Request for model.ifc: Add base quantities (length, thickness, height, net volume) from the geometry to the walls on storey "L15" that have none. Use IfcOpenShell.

First a look at what the model holds.

```python
import ifcopenshell
import ifcopenshell.util.element
import ifcopenshell.util.unit

model = ifcopenshell.open("model.ifc")
print(model.schema)
for unit_type in ("LENGTHUNIT", "AREAUNIT", "VOLUMEUNIT"):
    print(unit_type, ifcopenshell.util.unit.calculate_unit_scale(model, unit_type))
storey = next(s for s in model.by_type("IfcBuildingStorey") if s.Name == "L15")
walls = [e for e in ifcopenshell.util.element.get_decomposition(storey) if e.is_a("IfcWall")]
for e in sorted(walls, key=lambda e: e.id()):
    print(e.id(), e.is_a(), e.Name, list(ifcopenshell.util.element.get_psets(e, qtos_only=True)), sep=" | ")
```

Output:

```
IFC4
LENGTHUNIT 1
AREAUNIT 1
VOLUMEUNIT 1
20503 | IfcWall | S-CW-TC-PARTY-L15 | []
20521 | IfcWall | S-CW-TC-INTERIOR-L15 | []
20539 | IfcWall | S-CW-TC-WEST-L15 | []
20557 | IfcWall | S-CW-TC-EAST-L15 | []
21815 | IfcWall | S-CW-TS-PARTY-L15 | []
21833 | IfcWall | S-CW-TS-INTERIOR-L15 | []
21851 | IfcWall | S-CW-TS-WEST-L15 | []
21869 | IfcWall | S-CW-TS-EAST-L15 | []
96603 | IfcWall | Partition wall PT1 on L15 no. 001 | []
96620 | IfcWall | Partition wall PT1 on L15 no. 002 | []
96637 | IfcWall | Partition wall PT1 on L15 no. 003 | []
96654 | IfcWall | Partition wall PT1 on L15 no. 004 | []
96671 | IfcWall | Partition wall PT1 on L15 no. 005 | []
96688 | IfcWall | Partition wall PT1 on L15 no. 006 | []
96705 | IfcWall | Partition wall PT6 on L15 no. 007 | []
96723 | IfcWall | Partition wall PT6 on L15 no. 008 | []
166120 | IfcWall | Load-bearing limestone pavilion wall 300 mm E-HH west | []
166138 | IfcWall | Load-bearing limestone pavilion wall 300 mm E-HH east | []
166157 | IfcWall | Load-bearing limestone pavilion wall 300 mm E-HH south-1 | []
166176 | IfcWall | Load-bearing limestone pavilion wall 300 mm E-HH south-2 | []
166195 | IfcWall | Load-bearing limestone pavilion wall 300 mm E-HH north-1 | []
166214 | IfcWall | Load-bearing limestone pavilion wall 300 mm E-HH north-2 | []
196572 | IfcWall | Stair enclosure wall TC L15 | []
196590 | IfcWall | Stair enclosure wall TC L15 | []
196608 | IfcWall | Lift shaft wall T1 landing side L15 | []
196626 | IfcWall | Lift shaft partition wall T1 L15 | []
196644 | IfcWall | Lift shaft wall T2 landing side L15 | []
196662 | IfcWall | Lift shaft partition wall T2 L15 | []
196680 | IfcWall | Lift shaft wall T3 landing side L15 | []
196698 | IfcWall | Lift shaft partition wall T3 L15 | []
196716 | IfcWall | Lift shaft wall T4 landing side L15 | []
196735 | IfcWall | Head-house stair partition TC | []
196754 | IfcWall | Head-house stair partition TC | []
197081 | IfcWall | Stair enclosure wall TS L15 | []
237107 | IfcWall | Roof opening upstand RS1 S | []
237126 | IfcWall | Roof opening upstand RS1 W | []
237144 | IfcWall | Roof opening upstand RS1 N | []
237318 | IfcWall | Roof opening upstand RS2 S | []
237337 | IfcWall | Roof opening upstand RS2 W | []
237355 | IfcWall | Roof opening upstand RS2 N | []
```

```python
import ifcopenshell
import ifcopenshell.api.pset
import ifcopenshell.geom
import ifcopenshell.util.element
import ifcopenshell.util.shape
import ifcopenshell.util.unit

model = ifcopenshell.open("model.ifc")
unit_scale = ifcopenshell.util.unit.calculate_unit_scale(model)
volume_scale = ifcopenshell.util.unit.calculate_unit_scale(model, "VOLUMEUNIT")
settings = ifcopenshell.geom.settings()

storey = next(s for s in model.by_type("IfcBuildingStorey") if s.Name == "L15")
walls = [e for e in ifcopenshell.util.element.get_decomposition(storey) if e.is_a("IfcWall")]

for e in sorted(walls, key=lambda e: e.id()):
    if ifcopenshell.util.element.get_psets(e, qtos_only=True, should_inherit=False):
        continue
    # Geometry comes back in metres, in the element's own axes.
    shape = ifcopenshell.geom.create_shape(settings, e)
    values = {
        "Length": ifcopenshell.util.shape.get_x(shape.geometry) / unit_scale,
        "Width": ifcopenshell.util.shape.get_y(shape.geometry) / unit_scale,
        "Height": ifcopenshell.util.shape.get_z(shape.geometry) / unit_scale,
        "NetVolume": ifcopenshell.util.shape.get_volume(shape.geometry) / volume_scale,
    }
    qto = ifcopenshell.api.pset.add_qto(model, product=e, name="Qto_WallBaseQuantities")
    ifcopenshell.api.pset.edit_qto(model, qto=qto, properties=values)
    print(e.id(), {k: round(v, 3) for k, v in values.items()})

model.write("model_v2.ifc")
```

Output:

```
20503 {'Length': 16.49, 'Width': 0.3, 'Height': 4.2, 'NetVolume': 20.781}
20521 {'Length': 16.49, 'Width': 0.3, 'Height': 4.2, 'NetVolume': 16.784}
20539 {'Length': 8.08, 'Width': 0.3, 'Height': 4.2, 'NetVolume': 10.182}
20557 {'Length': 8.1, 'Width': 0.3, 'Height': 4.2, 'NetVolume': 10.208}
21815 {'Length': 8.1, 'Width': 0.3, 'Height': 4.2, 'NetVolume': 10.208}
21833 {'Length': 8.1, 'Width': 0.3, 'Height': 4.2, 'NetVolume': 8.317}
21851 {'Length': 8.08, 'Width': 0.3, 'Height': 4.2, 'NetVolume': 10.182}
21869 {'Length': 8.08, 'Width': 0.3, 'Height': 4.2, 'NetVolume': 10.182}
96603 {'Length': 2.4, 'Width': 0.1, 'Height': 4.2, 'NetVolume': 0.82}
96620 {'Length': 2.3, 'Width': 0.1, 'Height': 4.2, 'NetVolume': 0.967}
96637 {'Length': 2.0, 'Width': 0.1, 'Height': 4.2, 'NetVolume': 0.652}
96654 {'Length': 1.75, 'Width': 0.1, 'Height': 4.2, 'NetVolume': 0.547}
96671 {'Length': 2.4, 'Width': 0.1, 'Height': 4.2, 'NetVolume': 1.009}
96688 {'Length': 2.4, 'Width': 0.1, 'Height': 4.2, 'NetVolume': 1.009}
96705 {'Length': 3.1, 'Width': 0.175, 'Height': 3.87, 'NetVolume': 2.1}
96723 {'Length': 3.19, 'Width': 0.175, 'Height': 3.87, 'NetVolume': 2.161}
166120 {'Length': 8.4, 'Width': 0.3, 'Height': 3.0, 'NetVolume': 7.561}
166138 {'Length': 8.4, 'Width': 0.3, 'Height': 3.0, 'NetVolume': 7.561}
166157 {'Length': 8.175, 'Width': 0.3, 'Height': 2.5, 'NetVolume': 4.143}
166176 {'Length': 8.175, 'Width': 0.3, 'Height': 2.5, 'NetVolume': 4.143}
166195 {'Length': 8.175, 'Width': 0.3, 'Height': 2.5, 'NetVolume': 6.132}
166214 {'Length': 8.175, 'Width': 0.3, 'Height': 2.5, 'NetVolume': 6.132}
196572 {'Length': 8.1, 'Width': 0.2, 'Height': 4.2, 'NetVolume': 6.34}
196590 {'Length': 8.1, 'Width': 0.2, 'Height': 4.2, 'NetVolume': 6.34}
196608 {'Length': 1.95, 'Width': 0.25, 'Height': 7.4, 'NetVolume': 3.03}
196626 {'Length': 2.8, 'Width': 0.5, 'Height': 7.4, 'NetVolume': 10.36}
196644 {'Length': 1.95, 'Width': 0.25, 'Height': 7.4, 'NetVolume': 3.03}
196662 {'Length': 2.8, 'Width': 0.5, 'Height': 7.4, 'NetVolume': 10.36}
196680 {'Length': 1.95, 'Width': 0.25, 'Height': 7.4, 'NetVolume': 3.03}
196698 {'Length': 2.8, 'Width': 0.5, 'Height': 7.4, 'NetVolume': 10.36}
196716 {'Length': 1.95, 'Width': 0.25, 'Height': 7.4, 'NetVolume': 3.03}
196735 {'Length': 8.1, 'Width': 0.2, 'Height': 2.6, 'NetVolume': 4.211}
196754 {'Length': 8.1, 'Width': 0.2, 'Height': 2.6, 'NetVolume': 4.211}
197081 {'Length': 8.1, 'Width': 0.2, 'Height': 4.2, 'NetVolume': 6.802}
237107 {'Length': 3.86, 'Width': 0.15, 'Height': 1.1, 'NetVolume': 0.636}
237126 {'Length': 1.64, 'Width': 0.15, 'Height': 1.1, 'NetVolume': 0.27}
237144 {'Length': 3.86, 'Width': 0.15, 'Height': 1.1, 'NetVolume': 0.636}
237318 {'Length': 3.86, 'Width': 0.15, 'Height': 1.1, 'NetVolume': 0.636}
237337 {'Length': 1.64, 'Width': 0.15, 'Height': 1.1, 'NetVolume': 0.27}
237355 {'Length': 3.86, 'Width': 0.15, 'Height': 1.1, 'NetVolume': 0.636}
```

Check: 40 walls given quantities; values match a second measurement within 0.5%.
